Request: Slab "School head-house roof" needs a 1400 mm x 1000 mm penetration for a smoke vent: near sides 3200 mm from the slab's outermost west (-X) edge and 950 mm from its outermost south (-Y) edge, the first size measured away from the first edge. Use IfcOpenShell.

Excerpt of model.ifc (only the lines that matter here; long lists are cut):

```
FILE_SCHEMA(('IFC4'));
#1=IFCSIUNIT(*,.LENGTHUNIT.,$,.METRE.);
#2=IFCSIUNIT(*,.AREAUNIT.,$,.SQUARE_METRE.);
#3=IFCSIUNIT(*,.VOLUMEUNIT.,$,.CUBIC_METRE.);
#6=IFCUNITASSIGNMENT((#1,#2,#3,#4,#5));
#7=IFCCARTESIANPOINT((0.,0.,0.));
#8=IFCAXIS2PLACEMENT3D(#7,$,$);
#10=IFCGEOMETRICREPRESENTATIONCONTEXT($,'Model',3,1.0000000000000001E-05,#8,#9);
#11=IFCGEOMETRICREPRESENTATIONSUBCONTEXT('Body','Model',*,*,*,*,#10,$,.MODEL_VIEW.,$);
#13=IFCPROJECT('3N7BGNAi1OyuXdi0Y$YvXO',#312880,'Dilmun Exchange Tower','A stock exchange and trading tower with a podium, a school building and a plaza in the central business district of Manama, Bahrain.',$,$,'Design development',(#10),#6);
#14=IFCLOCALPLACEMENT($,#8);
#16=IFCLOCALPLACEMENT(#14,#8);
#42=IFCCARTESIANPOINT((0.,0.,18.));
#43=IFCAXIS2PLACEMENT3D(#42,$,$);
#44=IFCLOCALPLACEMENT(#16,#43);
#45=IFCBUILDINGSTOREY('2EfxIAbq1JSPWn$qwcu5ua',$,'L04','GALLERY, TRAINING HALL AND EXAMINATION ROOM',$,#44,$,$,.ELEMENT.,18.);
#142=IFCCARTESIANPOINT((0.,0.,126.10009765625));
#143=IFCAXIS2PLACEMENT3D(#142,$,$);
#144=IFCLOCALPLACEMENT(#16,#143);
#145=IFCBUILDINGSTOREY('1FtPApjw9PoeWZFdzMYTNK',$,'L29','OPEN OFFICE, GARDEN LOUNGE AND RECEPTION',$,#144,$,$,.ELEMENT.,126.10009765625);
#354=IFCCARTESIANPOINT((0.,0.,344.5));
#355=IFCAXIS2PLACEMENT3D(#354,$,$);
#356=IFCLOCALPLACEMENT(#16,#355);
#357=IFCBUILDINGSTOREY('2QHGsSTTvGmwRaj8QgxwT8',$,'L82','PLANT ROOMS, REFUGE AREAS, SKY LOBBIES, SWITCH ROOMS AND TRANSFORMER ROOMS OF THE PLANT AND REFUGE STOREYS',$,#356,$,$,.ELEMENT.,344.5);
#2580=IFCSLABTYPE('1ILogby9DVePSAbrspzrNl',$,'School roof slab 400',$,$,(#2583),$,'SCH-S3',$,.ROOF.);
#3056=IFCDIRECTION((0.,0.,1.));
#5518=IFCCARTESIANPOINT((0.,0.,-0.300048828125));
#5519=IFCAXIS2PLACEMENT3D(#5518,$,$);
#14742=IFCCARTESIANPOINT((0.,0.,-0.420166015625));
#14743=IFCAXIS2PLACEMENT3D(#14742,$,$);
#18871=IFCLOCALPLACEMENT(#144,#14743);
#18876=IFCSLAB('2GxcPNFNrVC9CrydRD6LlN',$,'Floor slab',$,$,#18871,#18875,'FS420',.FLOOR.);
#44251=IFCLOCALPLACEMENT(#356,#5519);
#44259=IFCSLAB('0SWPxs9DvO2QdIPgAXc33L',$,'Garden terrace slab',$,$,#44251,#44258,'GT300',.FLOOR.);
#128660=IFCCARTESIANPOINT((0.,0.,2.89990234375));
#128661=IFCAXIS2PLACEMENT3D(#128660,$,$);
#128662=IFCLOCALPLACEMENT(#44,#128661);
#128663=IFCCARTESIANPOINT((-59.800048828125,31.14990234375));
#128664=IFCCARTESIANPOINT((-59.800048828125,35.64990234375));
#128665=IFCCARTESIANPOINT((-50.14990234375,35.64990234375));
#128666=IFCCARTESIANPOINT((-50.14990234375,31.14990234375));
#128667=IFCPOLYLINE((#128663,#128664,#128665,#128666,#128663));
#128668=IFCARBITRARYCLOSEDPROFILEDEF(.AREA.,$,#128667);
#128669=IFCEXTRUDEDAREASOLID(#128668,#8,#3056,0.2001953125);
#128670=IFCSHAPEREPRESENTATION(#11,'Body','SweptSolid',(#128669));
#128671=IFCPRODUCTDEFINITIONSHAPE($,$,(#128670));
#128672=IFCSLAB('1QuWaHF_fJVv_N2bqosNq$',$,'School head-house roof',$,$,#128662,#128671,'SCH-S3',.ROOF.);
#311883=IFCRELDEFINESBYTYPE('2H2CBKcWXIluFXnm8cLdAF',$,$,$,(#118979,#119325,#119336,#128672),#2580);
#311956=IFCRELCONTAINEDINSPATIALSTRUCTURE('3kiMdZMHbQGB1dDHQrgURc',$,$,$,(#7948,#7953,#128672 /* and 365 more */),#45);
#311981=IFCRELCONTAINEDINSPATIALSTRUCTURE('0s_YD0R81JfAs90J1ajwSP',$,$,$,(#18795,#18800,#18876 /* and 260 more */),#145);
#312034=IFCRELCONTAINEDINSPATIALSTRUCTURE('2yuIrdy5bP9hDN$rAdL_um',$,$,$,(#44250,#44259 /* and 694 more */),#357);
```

```python
import numpy as np
import ifcopenshell
import ifcopenshell.api.feature
import ifcopenshell.api.geometry
import ifcopenshell.api.root
import ifcopenshell.geom
import ifcopenshell.util.placement
import ifcopenshell.util.representation
import ifcopenshell.util.shape
import ifcopenshell.util.unit

model = ifcopenshell.open("model.ifc")
unit_scale = ifcopenshell.util.unit.calculate_unit_scale(model)
settings = ifcopenshell.geom.settings()


def volume(element):
    """Net volume in cubic metres, openings subtracted."""
    shape = ifcopenshell.geom.create_shape(settings, element)
    return ifcopenshell.util.shape.get_volume(shape.geometry)


slab = model.by_id(128672)
before = volume(slab)

# Extent in the slab's own axes, in metres. The edges named are its -X and -Y sides.
slab_shape = ifcopenshell.geom.create_shape(settings, slab)
vertices = ifcopenshell.util.shape.get_vertices(slab_shape.geometry)
x_min, y_min, bottom = vertices.min(axis=0)
top = vertices[:, 2].max()

opening = ifcopenshell.api.root.create_entity(model, ifc_class="IfcOpeningElement", name="Smoke vent opening", predefined_type="OPENING")
context = ifcopenshell.util.representation.get_context(model, "Model", "Body", "MODEL_VIEW")
width, depth = 1.4, 1
outline = [(0.0, 0.0), (width, 0.0), (width, depth), (0.0, depth), (0.0, 0.0)]
# Overshoot both faces by 50 mm so the cut is clean.
shape = ifcopenshell.api.geometry.add_slab_representation(
    model, context=context, depth=top - bottom + 0.1, polyline=outline
)
ifcopenshell.api.geometry.assign_representation(model, product=opening, representation=shape)

matrix = ifcopenshell.util.placement.get_local_placement(slab.ObjectPlacement)
matrix[:, 3] = matrix @ np.append(np.array([x_min + 3.2, y_min + 0.95, bottom - 0.05]) / unit_scale, 1.0)
ifcopenshell.api.geometry.edit_object_placement(model, product=opening, matrix=matrix, is_si=False)
ifcopenshell.api.feature.add_feature(model, feature=opening, element=slab)

after = volume(slab)

print(f"slab volume {before:.3f} -> {after:.3f} m3")

model.write("model_updated.ifc")
```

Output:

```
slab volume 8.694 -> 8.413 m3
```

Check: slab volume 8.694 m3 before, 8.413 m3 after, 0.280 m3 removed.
